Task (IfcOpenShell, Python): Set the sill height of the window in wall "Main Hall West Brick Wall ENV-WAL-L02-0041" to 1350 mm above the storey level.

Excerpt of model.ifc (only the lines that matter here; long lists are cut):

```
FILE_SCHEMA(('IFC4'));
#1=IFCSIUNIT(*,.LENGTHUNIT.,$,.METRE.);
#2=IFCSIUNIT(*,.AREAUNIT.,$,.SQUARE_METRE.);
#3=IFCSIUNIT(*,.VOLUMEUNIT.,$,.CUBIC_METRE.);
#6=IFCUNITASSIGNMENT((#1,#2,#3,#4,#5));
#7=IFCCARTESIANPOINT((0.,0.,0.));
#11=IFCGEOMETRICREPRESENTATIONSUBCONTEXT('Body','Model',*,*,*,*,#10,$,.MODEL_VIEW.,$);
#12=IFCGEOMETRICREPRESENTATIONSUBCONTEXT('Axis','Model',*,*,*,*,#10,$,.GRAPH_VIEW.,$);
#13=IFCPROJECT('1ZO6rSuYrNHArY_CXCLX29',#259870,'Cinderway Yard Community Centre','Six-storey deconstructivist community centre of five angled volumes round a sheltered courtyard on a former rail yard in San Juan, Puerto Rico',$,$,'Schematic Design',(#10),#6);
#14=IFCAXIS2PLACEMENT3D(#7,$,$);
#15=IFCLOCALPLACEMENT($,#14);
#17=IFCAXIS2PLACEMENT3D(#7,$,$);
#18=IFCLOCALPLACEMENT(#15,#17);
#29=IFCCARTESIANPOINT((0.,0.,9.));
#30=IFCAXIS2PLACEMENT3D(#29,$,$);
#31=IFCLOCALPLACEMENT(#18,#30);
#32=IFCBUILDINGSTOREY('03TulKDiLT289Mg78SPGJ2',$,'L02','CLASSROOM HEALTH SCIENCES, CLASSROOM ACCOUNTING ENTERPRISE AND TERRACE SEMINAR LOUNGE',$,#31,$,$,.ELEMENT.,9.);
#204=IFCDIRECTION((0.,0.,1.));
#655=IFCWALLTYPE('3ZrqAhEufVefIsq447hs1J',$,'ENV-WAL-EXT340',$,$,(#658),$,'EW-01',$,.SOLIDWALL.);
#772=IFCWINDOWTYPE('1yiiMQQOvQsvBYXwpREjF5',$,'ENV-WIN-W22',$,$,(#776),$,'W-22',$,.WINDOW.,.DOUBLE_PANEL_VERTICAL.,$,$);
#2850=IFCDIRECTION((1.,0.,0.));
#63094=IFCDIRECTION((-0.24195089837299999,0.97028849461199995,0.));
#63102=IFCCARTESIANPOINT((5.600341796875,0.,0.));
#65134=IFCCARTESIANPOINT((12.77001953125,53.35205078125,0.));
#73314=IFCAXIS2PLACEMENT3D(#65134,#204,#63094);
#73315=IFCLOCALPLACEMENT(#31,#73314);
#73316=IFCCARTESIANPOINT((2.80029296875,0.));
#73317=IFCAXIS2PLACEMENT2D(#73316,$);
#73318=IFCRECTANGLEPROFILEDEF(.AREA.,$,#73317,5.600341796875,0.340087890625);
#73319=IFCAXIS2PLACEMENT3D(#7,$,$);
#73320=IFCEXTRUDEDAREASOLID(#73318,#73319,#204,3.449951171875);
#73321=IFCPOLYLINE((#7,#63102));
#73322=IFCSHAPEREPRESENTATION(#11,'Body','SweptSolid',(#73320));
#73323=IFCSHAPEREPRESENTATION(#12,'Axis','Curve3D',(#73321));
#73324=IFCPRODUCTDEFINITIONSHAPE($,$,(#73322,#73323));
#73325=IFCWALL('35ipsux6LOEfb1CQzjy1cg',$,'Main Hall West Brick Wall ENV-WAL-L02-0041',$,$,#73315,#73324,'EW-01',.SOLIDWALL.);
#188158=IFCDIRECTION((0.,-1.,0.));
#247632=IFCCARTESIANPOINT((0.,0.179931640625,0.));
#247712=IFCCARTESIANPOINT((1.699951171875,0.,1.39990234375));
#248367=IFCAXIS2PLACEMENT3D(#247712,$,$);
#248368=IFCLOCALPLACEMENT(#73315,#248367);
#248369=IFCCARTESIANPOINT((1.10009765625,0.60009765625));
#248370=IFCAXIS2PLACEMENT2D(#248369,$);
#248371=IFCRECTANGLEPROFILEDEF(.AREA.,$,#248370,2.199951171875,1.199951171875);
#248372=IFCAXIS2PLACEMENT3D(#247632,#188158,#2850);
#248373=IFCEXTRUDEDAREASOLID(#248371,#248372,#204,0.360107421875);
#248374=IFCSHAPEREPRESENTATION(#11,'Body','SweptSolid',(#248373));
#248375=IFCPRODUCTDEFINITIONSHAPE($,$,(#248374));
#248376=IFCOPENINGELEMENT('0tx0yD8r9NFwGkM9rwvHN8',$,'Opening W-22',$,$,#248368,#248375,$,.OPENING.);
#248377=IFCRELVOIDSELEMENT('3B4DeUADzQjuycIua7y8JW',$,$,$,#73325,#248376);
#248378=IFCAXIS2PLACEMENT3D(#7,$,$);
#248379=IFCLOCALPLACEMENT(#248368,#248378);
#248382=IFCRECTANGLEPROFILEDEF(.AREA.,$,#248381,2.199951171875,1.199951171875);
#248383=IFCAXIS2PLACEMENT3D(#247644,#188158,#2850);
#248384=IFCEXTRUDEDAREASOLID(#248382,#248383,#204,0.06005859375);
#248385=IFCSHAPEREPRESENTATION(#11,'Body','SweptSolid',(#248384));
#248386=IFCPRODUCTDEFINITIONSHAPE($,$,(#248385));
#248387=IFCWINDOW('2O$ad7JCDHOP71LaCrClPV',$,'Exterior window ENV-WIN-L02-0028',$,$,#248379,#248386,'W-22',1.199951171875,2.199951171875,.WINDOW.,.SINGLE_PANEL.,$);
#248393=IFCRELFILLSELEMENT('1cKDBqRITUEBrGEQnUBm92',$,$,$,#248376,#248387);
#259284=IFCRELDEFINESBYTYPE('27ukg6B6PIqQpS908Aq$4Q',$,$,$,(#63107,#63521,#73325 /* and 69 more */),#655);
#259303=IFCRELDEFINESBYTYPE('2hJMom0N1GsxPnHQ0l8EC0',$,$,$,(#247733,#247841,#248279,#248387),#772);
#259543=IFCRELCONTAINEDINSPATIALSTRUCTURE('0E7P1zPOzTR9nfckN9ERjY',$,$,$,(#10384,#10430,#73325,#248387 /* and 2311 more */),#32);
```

```python
import numpy as np
import ifcopenshell
import ifcopenshell.api.geometry
import ifcopenshell.geom
import ifcopenshell.util.element
import ifcopenshell.util.placement
import ifcopenshell.util.shape
import ifcopenshell.util.unit

model = ifcopenshell.open("model.ifc")
unit_scale = ifcopenshell.util.unit.calculate_unit_scale(model)

window = model.by_guid("2O$ad7JCDHOP71LaCrClPV")
opening = window.FillsVoids[0].RelatingOpeningElement
storey = ifcopenshell.util.element.get_container(window, ifc_class="IfcBuildingStorey")
level = ifcopenshell.util.placement.get_local_placement(storey.ObjectPlacement)[2, 3]

# The opening's origin need not be at the sill, so measure its lowest point.
shape = ifcopenshell.geom.create_shape(ifcopenshell.geom.settings(), opening)
bottom = ifcopenshell.util.shape.get_shape_bottom_elevation(shape, shape.geometry) / unit_scale
dz = level + 1.35 / unit_scale - bottom

shift = np.array([0.0, 0.0, dz])
# The window is placed relative to its opening, so it follows when the opening moves.
matrix = ifcopenshell.util.placement.get_local_placement(opening.ObjectPlacement)
matrix[:3, 3] += shift
ifcopenshell.api.geometry.edit_object_placement(
    model, product=opening, matrix=matrix, is_si=False, should_transform_children=True
)

print(f"moved by {dz * unit_scale:+.3f} m")

model.write("model_updated.ifc")
```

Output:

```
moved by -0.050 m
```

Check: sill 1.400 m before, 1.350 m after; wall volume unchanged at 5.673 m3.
